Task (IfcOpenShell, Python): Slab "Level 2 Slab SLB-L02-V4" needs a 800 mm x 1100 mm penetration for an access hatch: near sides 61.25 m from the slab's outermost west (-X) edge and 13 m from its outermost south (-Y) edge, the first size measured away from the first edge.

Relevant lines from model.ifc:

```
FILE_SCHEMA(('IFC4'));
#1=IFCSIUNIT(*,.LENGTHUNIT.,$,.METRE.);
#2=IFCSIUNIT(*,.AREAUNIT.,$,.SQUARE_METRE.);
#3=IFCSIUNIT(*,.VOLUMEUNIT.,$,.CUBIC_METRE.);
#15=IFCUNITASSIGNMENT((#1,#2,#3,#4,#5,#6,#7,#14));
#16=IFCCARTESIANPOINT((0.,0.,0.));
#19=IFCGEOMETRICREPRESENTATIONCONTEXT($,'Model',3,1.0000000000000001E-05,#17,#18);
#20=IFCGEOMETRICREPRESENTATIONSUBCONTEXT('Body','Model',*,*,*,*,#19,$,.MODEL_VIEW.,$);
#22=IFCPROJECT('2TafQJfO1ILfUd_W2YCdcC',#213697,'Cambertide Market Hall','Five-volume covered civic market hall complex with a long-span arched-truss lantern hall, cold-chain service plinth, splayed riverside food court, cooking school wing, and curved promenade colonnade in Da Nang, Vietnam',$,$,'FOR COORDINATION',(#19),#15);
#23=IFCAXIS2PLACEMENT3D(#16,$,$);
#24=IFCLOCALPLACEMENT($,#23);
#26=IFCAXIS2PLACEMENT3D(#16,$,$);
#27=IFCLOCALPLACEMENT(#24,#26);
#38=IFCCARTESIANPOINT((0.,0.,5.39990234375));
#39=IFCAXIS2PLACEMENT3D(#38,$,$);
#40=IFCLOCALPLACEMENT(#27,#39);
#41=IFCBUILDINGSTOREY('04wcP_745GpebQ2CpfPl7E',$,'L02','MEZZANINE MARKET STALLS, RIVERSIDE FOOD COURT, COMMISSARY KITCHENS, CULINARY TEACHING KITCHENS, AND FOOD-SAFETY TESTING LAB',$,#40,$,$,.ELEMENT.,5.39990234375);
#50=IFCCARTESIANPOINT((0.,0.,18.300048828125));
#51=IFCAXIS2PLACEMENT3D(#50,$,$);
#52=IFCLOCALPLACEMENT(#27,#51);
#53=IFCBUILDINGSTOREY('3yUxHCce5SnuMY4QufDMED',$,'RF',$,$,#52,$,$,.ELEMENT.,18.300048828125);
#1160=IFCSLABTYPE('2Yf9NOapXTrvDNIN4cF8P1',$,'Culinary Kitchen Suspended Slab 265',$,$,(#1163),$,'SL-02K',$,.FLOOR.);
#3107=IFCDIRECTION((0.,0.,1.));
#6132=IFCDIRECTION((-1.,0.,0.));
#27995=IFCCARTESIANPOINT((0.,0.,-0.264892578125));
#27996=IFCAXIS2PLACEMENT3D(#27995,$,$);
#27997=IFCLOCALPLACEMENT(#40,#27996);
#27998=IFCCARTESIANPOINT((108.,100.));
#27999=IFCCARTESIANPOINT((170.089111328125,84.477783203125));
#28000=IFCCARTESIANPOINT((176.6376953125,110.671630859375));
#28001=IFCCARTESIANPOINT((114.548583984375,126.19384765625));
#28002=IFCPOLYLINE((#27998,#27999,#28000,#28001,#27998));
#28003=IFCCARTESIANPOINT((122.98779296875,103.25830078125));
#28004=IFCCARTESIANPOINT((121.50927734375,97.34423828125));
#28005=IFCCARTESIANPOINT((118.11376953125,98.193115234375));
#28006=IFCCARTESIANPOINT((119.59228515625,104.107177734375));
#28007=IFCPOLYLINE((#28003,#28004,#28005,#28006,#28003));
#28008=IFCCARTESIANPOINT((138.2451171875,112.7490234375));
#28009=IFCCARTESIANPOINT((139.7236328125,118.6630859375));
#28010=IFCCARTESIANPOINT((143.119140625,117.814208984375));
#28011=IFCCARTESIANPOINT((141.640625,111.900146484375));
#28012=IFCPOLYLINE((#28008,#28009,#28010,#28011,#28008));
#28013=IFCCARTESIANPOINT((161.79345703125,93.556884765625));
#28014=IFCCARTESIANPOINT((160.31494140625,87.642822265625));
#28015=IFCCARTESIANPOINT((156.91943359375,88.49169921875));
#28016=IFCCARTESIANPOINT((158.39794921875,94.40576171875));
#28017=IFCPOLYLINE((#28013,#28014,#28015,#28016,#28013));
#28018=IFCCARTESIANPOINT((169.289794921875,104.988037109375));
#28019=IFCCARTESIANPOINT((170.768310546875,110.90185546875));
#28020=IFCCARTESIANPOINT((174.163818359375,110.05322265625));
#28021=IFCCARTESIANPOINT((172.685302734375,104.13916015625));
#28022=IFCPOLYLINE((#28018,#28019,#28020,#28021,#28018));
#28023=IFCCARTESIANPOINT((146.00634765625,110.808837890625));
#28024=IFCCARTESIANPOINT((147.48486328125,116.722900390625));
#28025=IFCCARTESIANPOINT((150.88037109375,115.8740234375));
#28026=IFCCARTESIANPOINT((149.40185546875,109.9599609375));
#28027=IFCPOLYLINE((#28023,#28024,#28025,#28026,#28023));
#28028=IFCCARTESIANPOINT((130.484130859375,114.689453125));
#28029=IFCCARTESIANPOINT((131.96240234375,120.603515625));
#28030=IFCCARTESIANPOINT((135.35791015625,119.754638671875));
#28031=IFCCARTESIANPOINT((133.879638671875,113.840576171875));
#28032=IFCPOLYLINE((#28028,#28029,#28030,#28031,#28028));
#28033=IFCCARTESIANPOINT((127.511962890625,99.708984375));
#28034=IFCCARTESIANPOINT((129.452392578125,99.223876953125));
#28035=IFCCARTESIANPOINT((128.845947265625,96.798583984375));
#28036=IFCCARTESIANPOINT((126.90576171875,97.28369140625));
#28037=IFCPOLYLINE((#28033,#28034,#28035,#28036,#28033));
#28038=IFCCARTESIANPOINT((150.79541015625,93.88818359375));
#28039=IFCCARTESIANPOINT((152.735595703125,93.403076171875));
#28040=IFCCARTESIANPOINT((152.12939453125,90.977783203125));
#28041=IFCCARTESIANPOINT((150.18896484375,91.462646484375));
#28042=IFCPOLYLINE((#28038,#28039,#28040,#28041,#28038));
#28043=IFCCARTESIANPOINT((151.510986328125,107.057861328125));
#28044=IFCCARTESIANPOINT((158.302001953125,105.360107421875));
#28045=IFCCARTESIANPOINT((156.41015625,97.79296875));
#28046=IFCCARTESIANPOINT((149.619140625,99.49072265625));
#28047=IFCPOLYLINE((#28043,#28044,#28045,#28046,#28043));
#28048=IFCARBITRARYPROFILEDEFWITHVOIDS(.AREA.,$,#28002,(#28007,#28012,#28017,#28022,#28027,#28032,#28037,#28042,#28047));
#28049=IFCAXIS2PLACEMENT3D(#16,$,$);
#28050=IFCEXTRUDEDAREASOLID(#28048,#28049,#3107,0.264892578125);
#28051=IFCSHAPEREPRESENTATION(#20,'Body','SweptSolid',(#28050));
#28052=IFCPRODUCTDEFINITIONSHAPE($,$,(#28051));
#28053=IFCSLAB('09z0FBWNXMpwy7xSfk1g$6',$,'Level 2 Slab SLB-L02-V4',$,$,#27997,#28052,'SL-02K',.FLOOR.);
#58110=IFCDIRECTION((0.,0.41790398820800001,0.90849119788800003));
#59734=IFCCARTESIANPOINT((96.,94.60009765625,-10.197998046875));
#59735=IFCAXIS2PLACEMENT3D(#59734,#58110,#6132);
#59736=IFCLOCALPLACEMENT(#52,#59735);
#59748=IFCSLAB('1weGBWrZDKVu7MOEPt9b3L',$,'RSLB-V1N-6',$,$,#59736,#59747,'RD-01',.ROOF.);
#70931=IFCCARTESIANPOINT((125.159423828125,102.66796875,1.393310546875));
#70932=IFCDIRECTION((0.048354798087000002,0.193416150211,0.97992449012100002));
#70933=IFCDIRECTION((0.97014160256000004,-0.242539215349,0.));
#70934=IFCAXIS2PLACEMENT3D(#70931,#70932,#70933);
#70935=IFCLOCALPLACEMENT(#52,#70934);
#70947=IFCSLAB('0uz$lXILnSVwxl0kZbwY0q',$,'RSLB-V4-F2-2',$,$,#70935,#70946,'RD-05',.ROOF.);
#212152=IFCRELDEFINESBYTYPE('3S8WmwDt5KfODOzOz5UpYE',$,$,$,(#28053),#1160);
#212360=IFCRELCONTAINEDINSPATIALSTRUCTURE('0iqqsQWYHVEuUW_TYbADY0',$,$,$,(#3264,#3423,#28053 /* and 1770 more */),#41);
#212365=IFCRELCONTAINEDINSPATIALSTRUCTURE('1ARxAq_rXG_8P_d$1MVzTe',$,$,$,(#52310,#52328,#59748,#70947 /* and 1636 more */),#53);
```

```python
import numpy as np
import ifcopenshell
import ifcopenshell.api.feature
import ifcopenshell.api.geometry
import ifcopenshell.api.root
import ifcopenshell.geom
import ifcopenshell.util.placement
import ifcopenshell.util.representation
import ifcopenshell.util.shape
import ifcopenshell.util.unit

model = ifcopenshell.open("model.ifc")
unit_scale = ifcopenshell.util.unit.calculate_unit_scale(model)
settings = ifcopenshell.geom.settings()


def volume(element):
    """Net volume in cubic metres, openings subtracted."""
    shape = ifcopenshell.geom.create_shape(settings, element)
    return ifcopenshell.util.shape.get_volume(shape.geometry)


slab = model.by_id(28053)
before = volume(slab)

# Extent in the slab's own axes, in metres. The edges named are its -X and -Y sides.
slab_shape = ifcopenshell.geom.create_shape(settings, slab)
vertices = ifcopenshell.util.shape.get_vertices(slab_shape.geometry)
x_min, y_min, bottom = vertices.min(axis=0)
top = vertices[:, 2].max()

opening = ifcopenshell.api.root.create_entity(model, ifc_class="IfcOpeningElement", name="Access hatch opening", predefined_type="OPENING")
context = ifcopenshell.util.representation.get_context(model, "Model", "Body", "MODEL_VIEW")
width, depth = 0.8, 1.1
outline = [(0.0, 0.0), (width, 0.0), (width, depth), (0.0, depth), (0.0, 0.0)]
# Overshoot both faces by 50 mm so the cut is clean.
shape = ifcopenshell.api.geometry.add_slab_representation(
    model, context=context, depth=top - bottom + 0.1, polyline=outline
)
ifcopenshell.api.geometry.assign_representation(model, product=opening, representation=shape)

matrix = ifcopenshell.util.placement.get_local_placement(slab.ObjectPlacement)
matrix[:, 3] = matrix @ np.append(np.array([x_min + 61.25, y_min + 13, bottom - 0.05]) / unit_scale, 1.0)
ifcopenshell.api.geometry.edit_object_placement(model, product=opening, matrix=matrix, is_si=False)
ifcopenshell.api.feature.add_feature(model, feature=opening, element=slab)

after = volume(slab)

print(f"slab volume {before:.3f} -> {after:.3f} m3")

model.write("model_edited.ifc")
```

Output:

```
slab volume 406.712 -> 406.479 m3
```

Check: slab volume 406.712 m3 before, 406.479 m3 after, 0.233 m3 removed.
